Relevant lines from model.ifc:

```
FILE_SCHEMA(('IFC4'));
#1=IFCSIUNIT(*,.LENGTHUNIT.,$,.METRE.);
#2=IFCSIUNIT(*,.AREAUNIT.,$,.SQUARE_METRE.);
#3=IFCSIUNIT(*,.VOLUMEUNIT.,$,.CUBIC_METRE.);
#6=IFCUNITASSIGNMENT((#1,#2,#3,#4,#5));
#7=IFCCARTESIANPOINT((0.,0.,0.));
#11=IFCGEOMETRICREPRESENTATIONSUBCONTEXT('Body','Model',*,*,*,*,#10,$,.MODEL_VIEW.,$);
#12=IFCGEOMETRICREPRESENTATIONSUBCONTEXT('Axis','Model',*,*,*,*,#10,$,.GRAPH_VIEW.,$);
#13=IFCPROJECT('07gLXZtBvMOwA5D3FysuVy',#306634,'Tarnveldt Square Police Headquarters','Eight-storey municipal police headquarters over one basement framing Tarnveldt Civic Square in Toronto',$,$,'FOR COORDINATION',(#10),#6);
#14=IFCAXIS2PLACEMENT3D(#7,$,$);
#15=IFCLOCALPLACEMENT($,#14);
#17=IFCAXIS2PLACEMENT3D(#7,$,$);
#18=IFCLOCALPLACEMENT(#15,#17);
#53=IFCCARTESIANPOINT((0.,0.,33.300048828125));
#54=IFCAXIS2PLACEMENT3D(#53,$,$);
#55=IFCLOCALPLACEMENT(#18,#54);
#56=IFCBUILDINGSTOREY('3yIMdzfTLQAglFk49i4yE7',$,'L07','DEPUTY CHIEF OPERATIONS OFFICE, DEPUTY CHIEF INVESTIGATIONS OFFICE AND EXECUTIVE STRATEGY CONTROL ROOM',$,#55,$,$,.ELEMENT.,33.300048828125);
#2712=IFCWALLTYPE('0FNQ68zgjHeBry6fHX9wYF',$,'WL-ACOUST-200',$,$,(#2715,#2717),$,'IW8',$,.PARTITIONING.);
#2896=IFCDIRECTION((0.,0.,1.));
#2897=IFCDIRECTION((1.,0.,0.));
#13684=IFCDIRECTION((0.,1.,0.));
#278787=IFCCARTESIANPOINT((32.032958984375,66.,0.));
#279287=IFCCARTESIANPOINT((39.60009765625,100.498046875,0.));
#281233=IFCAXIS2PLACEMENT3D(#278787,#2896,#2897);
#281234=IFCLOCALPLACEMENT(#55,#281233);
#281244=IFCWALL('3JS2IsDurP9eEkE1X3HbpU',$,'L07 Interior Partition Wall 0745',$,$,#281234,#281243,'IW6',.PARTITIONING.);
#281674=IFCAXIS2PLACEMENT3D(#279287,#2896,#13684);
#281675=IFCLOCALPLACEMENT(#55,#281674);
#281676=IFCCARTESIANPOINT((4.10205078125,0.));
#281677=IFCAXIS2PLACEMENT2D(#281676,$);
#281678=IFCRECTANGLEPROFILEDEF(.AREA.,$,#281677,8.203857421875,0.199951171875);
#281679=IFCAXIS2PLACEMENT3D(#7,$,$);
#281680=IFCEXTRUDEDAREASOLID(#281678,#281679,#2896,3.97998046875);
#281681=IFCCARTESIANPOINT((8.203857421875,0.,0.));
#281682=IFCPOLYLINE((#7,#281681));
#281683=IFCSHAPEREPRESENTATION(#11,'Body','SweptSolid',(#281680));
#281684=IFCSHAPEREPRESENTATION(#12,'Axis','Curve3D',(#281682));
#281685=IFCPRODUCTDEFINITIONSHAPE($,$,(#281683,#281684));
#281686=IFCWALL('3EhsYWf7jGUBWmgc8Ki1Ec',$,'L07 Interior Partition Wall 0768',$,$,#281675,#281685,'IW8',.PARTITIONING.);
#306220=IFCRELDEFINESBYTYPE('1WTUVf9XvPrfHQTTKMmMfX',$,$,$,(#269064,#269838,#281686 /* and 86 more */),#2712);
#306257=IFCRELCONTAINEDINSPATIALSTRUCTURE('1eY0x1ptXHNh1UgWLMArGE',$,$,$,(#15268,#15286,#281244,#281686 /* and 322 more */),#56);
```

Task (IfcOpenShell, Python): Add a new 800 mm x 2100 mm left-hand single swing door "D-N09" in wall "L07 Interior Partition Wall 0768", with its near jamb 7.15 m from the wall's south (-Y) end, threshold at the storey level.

```python
import numpy as np
import ifcopenshell
import ifcopenshell.api.feature
import ifcopenshell.api.geometry
import ifcopenshell.api.root
import ifcopenshell.api.spatial
import ifcopenshell.geom
import ifcopenshell.util.element
import ifcopenshell.util.placement
import ifcopenshell.util.representation
import ifcopenshell.util.shape
import ifcopenshell.util.unit

model = ifcopenshell.open("model.ifc")
unit_scale = ifcopenshell.util.unit.calculate_unit_scale(model)
settings = ifcopenshell.geom.settings()


def volume(element):
    """Net volume in cubic metres, openings subtracted."""
    shape = ifcopenshell.geom.create_shape(settings, element)
    return ifcopenshell.util.shape.get_volume(shape.geometry)


wall = model.by_guid("3EhsYWf7jGUBWmgc8Ki1Ec")
storey = ifcopenshell.util.element.get_container(wall, ifc_class="IfcBuildingStorey")
context = ifcopenshell.util.representation.get_context(model, "Model", "Body", "MODEL_VIEW")
before = volume(wall)

width, height, from_end, sill = 0.8, 2.1, 7.15, 0.0  # metres

# The wall runs along its own X axis, and the end named is its -X end.
wall_shape = ifcopenshell.geom.create_shape(settings, wall)
x, y, z = ifcopenshell.util.shape.get_vertices(wall_shape.geometry).T
start = x.min() + from_end
face, thickness = float(y.min()), float(y.max() - y.min())
wall_matrix = ifcopenshell.util.placement.get_local_placement(wall.ObjectPlacement)
level = ifcopenshell.util.placement.get_local_placement(storey.ObjectPlacement)[2, 3]


def in_wall(x, y):
    """Placement at x, y metres in the wall's axes, at sill height."""
    matrix = wall_matrix.copy()
    matrix[:, 3] = wall_matrix @ np.array([x / unit_scale, y / unit_scale, 0.0, 1.0])
    matrix[2, 3] = level + sill / unit_scale
    return matrix


# Opening: a box that overshoots both wall faces by 50 mm.
opening = ifcopenshell.api.root.create_entity(model, ifc_class="IfcOpeningElement", predefined_type="OPENING")
box = ifcopenshell.api.geometry.add_wall_representation(
    model, context=context, length=width, height=height, thickness=thickness + 0.1
)
ifcopenshell.api.geometry.assign_representation(model, product=opening, representation=box)
ifcopenshell.api.geometry.edit_object_placement(model, product=opening, matrix=in_wall(start, face - 0.05), is_si=False)
ifcopenshell.api.feature.add_feature(model, feature=opening, element=wall)

door = ifcopenshell.api.root.create_entity(model, ifc_class="IfcDoor", name="D-N09", predefined_type="DOOR")
door.OverallWidth, door.OverallHeight = width / unit_scale, height / unit_scale
door.OperationType = "SINGLE_SWING_LEFT"
body = ifcopenshell.api.geometry.add_door_representation(
    model,
    context=context,
    overall_width=door.OverallWidth,
    overall_height=door.OverallHeight,
    operation_type="SINGLE_SWING_LEFT",
    lining_properties={"LiningDepth": thickness / unit_scale, "ThresholdDepth": thickness / unit_scale},
)
ifcopenshell.api.geometry.assign_representation(model, product=door, representation=body)
ifcopenshell.api.spatial.assign_container(model, products=[door], relating_structure=storey)
ifcopenshell.api.feature.add_filling(model, opening=opening, element=door)

# The lining spans the wall, so the door starts at the wall face.
ifcopenshell.api.geometry.edit_object_placement(model, product=door, matrix=in_wall(start, face), is_si=False)

after = volume(wall)

print(f"wall volume {before:.3f} -> {after:.3f} m3")

model.write("model_updated.ifc")
```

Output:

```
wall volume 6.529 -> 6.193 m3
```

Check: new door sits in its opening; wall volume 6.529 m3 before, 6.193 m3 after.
